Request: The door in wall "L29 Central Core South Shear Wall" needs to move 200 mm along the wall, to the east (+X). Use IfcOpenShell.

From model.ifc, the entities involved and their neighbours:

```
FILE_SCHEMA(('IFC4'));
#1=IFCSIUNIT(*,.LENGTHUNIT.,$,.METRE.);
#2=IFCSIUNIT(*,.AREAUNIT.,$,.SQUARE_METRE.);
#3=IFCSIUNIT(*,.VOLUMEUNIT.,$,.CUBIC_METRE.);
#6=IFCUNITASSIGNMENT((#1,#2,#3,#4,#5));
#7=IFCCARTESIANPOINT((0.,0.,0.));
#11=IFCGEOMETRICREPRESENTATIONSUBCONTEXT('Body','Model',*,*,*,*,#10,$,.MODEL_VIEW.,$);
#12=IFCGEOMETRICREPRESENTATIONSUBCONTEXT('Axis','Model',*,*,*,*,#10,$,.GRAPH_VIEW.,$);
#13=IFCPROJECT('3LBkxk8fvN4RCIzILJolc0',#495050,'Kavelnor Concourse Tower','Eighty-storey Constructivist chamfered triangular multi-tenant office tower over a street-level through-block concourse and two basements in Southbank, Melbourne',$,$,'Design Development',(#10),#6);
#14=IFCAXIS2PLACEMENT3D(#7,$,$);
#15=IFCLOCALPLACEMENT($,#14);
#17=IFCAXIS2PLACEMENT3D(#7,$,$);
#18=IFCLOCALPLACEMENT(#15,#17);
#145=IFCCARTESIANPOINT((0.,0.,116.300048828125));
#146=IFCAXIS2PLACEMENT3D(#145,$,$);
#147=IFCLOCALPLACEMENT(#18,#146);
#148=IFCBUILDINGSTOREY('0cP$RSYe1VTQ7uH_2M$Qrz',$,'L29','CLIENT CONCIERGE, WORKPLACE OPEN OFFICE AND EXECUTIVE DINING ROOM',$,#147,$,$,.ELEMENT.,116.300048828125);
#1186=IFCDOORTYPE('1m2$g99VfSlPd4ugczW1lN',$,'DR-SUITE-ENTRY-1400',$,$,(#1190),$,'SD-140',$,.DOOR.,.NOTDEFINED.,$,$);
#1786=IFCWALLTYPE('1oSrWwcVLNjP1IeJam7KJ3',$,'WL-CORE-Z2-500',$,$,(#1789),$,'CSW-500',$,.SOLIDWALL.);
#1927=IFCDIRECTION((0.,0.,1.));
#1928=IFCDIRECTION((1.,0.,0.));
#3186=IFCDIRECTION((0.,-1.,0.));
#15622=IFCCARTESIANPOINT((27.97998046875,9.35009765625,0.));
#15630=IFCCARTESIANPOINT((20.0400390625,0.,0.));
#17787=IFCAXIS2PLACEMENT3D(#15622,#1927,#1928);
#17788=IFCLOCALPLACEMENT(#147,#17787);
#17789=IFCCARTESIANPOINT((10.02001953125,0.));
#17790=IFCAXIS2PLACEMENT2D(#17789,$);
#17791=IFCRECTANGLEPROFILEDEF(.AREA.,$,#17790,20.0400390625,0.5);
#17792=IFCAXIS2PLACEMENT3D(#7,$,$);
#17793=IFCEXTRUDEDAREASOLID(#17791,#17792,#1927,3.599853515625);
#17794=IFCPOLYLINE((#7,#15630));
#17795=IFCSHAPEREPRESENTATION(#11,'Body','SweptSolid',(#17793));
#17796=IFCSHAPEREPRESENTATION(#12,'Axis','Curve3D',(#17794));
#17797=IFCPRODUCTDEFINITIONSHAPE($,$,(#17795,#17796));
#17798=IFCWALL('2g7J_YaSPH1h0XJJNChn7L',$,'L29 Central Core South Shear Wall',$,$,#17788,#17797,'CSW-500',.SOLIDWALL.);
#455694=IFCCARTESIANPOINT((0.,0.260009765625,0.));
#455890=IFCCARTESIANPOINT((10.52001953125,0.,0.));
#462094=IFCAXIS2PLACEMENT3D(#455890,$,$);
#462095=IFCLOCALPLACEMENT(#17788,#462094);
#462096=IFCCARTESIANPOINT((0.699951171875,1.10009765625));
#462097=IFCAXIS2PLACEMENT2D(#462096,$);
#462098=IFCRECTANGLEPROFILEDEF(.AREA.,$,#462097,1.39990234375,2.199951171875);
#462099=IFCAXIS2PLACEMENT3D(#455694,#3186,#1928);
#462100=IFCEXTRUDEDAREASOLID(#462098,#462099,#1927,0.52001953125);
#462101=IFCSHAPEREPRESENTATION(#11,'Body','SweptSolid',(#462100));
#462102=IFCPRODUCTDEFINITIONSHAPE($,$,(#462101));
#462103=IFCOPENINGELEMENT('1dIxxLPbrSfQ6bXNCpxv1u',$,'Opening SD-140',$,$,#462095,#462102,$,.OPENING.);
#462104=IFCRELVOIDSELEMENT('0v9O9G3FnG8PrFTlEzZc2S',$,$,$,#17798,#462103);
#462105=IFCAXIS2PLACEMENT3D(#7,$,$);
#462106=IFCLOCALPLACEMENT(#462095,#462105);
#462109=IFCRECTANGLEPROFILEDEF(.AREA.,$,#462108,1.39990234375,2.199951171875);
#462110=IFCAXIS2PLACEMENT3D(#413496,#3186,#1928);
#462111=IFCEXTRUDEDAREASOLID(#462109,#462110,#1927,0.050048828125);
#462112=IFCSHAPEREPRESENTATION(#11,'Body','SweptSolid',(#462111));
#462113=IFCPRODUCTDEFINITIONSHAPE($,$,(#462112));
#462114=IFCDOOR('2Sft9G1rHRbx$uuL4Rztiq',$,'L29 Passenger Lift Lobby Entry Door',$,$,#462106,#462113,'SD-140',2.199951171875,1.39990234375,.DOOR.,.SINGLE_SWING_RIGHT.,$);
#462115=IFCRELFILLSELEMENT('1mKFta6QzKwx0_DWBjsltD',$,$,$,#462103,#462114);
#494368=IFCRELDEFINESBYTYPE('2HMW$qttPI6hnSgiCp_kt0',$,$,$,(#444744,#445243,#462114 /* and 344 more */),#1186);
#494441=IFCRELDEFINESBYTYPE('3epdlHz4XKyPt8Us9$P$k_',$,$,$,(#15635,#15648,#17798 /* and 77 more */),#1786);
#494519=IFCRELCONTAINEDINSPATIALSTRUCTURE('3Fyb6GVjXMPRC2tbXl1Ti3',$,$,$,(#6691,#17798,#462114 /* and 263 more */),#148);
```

```python
import ifcopenshell
import ifcopenshell.api.geometry
import ifcopenshell.util.placement

model = ifcopenshell.open("model.ifc")

door = model.by_guid("2Sft9G1rHRbx$uuL4Rztiq")
opening = door.FillsVoids[0].RelatingOpeningElement
wall = opening.VoidsElements[0].RelatingBuildingElement

wall_matrix = ifcopenshell.util.placement.get_local_placement(wall.ObjectPlacement)
shift = wall_matrix[:3, 0] * 0.2
before = ifcopenshell.util.placement.get_local_placement(door.ObjectPlacement)[:3, 3].copy()

# The door is placed relative to its opening, so it follows when the opening moves.
matrix = ifcopenshell.util.placement.get_local_placement(opening.ObjectPlacement)
matrix[:3, 3] += shift
ifcopenshell.api.geometry.edit_object_placement(
    model, product=opening, matrix=matrix, is_si=False, should_transform_children=True
)

after = ifcopenshell.util.placement.get_local_placement(door.ObjectPlacement)[:3, 3]
print("door moved by", (after - before).round(3) + 0.0)

model.write("model_updated.ifc")
```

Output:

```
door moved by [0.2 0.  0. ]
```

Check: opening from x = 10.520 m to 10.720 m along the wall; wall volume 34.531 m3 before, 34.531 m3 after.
